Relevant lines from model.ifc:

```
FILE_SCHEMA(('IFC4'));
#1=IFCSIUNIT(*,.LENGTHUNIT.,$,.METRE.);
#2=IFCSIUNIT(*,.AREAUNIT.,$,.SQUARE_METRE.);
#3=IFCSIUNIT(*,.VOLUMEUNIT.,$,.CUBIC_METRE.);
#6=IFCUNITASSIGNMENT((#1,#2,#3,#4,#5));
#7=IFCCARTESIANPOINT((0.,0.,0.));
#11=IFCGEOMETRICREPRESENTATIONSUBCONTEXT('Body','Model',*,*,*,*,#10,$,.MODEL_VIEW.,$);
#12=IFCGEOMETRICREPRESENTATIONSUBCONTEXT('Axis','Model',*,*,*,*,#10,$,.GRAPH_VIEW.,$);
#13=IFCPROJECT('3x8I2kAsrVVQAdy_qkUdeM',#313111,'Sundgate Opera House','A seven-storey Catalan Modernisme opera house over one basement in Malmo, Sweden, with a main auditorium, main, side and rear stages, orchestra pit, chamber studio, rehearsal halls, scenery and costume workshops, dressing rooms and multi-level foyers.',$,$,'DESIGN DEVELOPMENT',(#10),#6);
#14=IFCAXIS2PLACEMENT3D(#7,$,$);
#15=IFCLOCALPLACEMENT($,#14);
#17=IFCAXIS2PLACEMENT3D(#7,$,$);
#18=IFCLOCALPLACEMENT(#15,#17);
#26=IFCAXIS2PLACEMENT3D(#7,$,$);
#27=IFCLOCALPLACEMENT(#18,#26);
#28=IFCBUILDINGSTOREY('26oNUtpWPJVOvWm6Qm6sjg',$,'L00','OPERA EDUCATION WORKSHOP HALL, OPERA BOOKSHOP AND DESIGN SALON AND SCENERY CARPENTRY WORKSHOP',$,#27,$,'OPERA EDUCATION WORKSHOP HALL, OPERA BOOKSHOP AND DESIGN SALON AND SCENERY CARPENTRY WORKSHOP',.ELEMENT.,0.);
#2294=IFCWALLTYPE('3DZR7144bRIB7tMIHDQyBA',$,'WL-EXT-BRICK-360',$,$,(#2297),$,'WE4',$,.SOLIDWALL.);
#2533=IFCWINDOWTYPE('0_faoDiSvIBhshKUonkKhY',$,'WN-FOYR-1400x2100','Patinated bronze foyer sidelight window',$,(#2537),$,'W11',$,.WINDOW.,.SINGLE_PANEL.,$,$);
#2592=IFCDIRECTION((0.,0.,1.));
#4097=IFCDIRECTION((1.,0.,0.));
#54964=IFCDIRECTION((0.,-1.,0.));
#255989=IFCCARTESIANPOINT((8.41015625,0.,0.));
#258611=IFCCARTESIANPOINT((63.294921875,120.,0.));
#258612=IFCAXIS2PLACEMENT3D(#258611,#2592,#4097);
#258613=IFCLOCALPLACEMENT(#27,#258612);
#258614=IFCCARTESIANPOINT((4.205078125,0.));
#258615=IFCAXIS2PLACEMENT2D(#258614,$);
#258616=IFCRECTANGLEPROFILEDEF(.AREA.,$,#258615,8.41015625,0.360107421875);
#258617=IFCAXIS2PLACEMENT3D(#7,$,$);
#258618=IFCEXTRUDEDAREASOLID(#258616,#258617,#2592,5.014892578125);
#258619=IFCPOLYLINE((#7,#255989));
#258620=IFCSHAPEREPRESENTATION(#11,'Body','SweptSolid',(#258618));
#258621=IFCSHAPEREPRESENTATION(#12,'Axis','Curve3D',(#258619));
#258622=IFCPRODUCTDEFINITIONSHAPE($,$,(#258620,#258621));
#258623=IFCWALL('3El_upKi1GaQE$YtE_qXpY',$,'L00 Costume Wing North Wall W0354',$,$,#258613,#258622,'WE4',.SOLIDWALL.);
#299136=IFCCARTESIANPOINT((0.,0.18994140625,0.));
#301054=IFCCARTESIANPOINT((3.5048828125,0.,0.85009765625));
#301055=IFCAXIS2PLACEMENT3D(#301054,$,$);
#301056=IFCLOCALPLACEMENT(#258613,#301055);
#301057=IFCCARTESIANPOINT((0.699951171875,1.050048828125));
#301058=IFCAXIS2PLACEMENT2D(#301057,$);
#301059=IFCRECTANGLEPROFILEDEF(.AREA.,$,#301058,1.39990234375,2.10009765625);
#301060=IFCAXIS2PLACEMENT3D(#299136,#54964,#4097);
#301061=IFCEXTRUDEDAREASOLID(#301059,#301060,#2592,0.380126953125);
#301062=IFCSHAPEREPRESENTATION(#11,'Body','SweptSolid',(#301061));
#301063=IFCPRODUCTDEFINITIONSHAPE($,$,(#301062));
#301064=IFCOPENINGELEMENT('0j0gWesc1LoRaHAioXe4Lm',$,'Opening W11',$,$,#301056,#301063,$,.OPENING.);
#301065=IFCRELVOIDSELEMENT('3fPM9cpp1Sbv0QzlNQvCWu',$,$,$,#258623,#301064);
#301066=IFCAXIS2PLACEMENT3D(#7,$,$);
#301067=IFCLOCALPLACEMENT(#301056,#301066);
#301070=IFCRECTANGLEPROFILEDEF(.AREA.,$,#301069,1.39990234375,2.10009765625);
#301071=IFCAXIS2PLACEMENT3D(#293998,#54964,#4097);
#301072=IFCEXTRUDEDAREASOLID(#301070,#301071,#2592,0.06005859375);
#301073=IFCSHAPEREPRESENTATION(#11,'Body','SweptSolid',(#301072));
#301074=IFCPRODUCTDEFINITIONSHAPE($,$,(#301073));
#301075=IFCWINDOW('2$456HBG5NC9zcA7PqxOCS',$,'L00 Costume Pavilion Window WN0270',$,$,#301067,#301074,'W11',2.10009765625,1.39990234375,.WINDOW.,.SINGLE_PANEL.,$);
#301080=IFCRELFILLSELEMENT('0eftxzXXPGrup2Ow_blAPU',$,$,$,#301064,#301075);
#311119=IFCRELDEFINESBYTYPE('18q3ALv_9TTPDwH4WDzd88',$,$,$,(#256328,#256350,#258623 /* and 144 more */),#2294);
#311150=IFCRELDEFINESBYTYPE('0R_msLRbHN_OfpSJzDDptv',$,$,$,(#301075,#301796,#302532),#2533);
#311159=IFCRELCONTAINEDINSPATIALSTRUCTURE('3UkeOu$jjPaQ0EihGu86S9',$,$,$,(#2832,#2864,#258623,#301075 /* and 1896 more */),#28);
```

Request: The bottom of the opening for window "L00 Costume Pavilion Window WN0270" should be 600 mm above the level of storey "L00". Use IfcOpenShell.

```python
import numpy as np
import ifcopenshell
import ifcopenshell.api.geometry
import ifcopenshell.geom
import ifcopenshell.util.element
import ifcopenshell.util.placement
import ifcopenshell.util.shape
import ifcopenshell.util.unit

model = ifcopenshell.open("model.ifc")
unit_scale = ifcopenshell.util.unit.calculate_unit_scale(model)

window = model.by_guid("2$456HBG5NC9zcA7PqxOCS")
opening = window.FillsVoids[0].RelatingOpeningElement
storey = ifcopenshell.util.element.get_container(window, ifc_class="IfcBuildingStorey")
level = ifcopenshell.util.placement.get_local_placement(storey.ObjectPlacement)[2, 3]

# The opening's origin need not be at the sill, so measure its lowest point.
shape = ifcopenshell.geom.create_shape(ifcopenshell.geom.settings(), opening)
bottom = ifcopenshell.util.shape.get_shape_bottom_elevation(shape, shape.geometry) / unit_scale
dz = level + 0.6 / unit_scale - bottom

shift = np.array([0.0, 0.0, dz])
# The window is placed relative to its opening, so it follows when the opening moves.
matrix = ifcopenshell.util.placement.get_local_placement(opening.ObjectPlacement)
matrix[:3, 3] += shift
ifcopenshell.api.geometry.edit_object_placement(
    model, product=opening, matrix=matrix, is_si=False, should_transform_children=True
)

print(f"moved by {dz * unit_scale:+.3f} m")

model.write("model_v2.ifc")
```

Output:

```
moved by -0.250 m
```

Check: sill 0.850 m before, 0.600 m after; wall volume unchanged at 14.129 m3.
